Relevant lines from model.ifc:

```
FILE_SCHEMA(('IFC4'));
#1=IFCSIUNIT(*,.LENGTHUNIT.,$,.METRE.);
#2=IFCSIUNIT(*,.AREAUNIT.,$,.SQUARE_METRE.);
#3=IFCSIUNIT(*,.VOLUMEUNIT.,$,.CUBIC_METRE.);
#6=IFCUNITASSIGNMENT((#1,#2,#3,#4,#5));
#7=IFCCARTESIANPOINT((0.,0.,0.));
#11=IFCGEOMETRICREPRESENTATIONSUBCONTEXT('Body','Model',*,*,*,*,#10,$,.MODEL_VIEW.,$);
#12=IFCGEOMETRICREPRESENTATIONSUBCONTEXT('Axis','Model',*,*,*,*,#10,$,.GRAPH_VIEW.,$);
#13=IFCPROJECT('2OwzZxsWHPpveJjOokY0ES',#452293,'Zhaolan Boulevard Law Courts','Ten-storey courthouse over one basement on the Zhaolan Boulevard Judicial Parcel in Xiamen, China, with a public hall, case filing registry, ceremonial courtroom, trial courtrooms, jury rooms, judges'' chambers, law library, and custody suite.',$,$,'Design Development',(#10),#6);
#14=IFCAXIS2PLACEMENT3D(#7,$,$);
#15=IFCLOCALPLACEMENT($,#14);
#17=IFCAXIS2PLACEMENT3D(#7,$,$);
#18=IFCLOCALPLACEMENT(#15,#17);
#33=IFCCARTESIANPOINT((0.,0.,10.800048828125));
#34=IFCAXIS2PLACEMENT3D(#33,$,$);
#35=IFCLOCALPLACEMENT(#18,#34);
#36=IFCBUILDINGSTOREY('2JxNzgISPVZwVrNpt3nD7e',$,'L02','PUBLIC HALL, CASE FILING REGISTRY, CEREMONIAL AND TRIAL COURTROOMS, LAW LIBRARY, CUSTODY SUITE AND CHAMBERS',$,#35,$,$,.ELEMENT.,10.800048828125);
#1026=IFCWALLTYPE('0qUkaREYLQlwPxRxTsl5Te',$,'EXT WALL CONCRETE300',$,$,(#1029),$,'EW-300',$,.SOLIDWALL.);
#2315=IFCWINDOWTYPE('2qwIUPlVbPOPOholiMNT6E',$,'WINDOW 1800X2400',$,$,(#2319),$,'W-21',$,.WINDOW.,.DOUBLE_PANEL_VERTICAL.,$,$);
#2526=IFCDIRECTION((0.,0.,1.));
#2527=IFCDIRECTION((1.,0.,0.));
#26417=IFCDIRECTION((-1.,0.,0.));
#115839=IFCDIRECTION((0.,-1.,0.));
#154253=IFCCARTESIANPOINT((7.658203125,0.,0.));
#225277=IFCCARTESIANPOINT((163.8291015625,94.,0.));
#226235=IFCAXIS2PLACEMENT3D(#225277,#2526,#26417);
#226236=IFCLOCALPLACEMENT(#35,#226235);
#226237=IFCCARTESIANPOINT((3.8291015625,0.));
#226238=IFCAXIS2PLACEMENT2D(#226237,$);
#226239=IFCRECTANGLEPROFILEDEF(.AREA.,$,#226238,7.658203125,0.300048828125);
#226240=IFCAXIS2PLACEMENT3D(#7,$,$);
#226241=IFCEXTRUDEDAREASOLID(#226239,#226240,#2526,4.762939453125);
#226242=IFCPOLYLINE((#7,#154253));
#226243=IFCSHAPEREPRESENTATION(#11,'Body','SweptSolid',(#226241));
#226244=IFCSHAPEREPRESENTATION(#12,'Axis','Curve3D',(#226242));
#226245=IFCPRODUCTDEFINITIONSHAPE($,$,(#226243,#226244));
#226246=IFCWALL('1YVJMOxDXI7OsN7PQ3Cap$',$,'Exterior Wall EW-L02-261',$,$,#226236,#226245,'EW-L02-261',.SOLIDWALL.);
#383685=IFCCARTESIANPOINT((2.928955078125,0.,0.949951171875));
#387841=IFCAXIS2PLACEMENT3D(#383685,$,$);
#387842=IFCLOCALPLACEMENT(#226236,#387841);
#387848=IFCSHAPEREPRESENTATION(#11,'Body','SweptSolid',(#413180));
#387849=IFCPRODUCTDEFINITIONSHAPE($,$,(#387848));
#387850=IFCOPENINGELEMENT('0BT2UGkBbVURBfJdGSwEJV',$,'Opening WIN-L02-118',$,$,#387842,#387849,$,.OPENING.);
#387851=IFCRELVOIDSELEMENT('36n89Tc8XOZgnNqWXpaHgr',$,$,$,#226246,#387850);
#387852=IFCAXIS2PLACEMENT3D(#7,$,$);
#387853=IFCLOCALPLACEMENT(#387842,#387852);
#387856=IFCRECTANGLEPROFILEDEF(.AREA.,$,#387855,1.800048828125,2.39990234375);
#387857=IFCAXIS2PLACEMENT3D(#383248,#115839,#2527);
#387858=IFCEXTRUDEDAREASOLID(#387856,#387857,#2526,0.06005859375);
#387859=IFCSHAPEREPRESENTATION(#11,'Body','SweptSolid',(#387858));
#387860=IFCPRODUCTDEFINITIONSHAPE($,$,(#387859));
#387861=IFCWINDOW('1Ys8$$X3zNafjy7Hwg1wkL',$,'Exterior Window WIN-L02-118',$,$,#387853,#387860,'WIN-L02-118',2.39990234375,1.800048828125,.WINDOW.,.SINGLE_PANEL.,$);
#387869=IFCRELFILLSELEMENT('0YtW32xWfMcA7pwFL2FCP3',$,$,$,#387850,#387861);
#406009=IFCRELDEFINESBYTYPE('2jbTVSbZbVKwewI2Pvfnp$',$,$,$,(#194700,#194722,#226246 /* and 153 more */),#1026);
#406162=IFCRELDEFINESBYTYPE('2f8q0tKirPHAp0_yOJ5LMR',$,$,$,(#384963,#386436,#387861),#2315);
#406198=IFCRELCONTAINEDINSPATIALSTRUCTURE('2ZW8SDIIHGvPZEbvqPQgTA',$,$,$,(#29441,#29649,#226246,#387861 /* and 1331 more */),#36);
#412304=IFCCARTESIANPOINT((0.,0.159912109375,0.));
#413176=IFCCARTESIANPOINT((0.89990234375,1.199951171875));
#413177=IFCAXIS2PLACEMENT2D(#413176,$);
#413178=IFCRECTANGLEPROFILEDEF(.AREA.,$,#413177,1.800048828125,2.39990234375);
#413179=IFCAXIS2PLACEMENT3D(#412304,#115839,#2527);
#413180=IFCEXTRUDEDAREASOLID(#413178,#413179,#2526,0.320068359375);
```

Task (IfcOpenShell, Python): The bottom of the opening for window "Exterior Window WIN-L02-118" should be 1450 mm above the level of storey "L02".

```python
import numpy as np
import ifcopenshell
import ifcopenshell.api.geometry
import ifcopenshell.geom
import ifcopenshell.util.element
import ifcopenshell.util.placement
import ifcopenshell.util.shape
import ifcopenshell.util.unit

model = ifcopenshell.open("model.ifc")
unit_scale = ifcopenshell.util.unit.calculate_unit_scale(model)

window = model.by_id(387861)
opening = window.FillsVoids[0].RelatingOpeningElement
storey = ifcopenshell.util.element.get_container(window, ifc_class="IfcBuildingStorey")
level = ifcopenshell.util.placement.get_local_placement(storey.ObjectPlacement)[2, 3]

# The opening's origin need not be at the sill, so measure its lowest point.
shape = ifcopenshell.geom.create_shape(ifcopenshell.geom.settings(), opening)
bottom = ifcopenshell.util.shape.get_shape_bottom_elevation(shape, shape.geometry) / unit_scale
dz = level + 1.45 / unit_scale - bottom

shift = np.array([0.0, 0.0, dz])
# The window is placed relative to its opening, so it follows when the opening moves.
matrix = ifcopenshell.util.placement.get_local_placement(opening.ObjectPlacement)
matrix[:3, 3] += shift
ifcopenshell.api.geometry.edit_object_placement(
    model, product=opening, matrix=matrix, is_si=False, should_transform_children=True
)

print(f"moved by {dz * unit_scale:+.3f} m")

model.write("model-out.ifc")
```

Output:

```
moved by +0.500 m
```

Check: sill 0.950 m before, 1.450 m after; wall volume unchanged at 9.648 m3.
